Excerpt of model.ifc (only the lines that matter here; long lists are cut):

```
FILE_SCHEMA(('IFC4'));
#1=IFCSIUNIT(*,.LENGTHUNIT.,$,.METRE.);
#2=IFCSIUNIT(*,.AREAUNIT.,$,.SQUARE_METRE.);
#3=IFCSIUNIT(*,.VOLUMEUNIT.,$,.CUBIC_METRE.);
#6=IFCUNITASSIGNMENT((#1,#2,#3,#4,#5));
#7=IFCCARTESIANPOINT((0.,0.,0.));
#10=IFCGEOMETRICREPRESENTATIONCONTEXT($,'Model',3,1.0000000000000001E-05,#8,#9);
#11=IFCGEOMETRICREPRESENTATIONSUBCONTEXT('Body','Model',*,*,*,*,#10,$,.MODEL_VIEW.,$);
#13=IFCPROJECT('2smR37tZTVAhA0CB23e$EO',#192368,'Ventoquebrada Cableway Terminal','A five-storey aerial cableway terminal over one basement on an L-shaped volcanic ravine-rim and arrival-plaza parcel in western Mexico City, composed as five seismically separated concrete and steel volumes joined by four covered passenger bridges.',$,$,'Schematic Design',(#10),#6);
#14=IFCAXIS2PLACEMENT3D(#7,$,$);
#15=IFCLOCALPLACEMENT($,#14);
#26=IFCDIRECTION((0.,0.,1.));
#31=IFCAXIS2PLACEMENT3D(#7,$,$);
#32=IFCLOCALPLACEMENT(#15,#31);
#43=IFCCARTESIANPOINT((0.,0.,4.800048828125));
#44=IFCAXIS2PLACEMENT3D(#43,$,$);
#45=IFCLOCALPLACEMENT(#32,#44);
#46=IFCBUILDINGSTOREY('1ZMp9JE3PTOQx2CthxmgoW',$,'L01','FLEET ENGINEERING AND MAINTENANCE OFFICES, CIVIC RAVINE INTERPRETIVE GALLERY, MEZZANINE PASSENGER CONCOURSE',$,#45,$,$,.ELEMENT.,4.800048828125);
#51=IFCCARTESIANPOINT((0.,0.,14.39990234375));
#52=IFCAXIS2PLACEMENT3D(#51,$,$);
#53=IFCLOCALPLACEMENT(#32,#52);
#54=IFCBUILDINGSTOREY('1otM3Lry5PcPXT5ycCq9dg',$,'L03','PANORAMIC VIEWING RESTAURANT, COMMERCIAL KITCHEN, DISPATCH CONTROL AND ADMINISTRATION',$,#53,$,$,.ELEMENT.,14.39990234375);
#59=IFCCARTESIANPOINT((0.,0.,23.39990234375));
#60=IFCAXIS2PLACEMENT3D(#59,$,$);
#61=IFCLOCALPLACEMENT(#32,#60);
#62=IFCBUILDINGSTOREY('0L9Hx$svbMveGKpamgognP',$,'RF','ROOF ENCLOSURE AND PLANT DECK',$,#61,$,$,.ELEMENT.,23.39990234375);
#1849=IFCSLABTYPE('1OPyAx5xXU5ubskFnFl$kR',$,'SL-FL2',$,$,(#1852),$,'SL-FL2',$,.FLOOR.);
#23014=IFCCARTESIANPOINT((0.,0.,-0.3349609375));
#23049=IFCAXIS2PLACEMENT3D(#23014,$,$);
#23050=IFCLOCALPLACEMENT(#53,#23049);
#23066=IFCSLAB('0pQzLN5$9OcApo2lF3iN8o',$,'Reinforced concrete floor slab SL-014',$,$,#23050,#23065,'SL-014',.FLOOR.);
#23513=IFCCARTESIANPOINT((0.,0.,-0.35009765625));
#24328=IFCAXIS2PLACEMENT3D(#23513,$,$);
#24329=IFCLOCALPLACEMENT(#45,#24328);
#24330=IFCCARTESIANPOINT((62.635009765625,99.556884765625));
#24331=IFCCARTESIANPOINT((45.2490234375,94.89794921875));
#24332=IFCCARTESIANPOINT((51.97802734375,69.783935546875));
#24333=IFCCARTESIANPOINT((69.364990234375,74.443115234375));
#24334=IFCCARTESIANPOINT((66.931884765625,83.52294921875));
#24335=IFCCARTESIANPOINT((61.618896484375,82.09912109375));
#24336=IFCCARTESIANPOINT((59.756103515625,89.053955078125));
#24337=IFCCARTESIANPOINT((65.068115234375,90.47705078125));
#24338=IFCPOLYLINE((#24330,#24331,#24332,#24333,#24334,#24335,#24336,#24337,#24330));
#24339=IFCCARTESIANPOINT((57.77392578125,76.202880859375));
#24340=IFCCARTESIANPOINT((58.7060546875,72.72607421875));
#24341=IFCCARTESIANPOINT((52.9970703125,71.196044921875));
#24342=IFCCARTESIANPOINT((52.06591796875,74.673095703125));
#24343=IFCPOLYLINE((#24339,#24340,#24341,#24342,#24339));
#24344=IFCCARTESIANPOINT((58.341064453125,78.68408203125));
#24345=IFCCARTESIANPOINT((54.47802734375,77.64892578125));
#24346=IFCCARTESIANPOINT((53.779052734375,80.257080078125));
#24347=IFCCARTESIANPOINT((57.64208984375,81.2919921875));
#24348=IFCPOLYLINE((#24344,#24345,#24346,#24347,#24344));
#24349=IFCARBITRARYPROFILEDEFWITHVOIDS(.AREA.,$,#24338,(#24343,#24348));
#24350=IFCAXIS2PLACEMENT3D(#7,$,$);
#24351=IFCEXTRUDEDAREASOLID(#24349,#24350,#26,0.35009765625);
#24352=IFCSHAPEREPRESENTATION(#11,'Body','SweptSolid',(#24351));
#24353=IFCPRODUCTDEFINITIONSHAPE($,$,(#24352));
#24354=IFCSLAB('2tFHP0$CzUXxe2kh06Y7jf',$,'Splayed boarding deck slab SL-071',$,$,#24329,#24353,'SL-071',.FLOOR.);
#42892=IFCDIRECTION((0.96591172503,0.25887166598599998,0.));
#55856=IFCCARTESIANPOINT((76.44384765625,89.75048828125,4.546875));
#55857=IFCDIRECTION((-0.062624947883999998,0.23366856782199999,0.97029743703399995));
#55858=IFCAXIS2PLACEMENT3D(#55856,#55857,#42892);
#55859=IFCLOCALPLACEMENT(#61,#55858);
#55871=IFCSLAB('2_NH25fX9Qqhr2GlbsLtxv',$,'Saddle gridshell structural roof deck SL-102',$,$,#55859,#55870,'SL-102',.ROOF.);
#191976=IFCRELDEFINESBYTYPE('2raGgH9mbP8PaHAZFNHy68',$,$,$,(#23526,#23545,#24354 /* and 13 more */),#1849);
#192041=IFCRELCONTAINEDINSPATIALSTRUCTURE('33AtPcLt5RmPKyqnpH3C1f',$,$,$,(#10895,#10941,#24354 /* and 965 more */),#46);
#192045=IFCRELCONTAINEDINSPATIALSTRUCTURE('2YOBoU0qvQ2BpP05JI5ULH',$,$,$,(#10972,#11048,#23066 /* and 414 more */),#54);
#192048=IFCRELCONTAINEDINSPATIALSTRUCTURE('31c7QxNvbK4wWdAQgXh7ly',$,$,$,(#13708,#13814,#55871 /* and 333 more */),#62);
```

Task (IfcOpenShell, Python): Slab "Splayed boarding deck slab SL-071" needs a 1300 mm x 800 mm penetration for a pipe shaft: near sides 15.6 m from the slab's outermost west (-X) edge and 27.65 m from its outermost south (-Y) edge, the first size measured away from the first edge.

```python
import numpy as np
import ifcopenshell
import ifcopenshell.api.feature
import ifcopenshell.api.geometry
import ifcopenshell.api.root
import ifcopenshell.geom
import ifcopenshell.util.placement
import ifcopenshell.util.representation
import ifcopenshell.util.shape
import ifcopenshell.util.unit

model = ifcopenshell.open("model.ifc")
unit_scale = ifcopenshell.util.unit.calculate_unit_scale(model)
settings = ifcopenshell.geom.settings()


def volume(element):
    """Net volume in cubic metres, openings subtracted."""
    shape = ifcopenshell.geom.create_shape(settings, element)
    return ifcopenshell.util.shape.get_volume(shape.geometry)


slab = model.by_guid("2tFHP0$CzUXxe2kh06Y7jf")
before = volume(slab)

# Extent in the slab's own axes, in metres. The edges named are its -X and -Y sides.
slab_shape = ifcopenshell.geom.create_shape(settings, slab)
vertices = ifcopenshell.util.shape.get_vertices(slab_shape.geometry)
x_min, y_min, bottom = vertices.min(axis=0)
top = vertices[:, 2].max()

opening = ifcopenshell.api.root.create_entity(model, ifc_class="IfcOpeningElement", name="Pipe shaft opening", predefined_type="OPENING")
context = ifcopenshell.util.representation.get_context(model, "Model", "Body", "MODEL_VIEW")
width, depth = 1.3, 0.8
outline = [(0.0, 0.0), (width, 0.0), (width, depth), (0.0, depth), (0.0, 0.0)]
# Overshoot both faces by 50 mm so the cut is clean.
shape = ifcopenshell.api.geometry.add_slab_representation(
    model, context=context, depth=top - bottom + 0.1, polyline=outline
)
ifcopenshell.api.geometry.assign_representation(model, product=opening, representation=shape)

matrix = ifcopenshell.util.placement.get_local_placement(slab.ObjectPlacement)
matrix[:, 3] = matrix @ np.append(np.array([x_min + 15.6, y_min + 27.65, bottom - 0.05]) / unit_scale, 1.0)
ifcopenshell.api.geometry.edit_object_placement(model, product=opening, matrix=matrix, is_si=False)
ifcopenshell.api.feature.add_feature(model, feature=opening, element=slab)

after = volume(slab)

print(f"slab volume {before:.3f} -> {after:.3f} m3")

model.write("model_edited.ifc")
```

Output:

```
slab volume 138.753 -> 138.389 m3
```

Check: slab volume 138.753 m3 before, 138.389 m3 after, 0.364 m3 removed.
